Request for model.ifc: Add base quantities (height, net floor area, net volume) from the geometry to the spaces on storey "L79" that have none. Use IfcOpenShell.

First a look at what the model holds.

```python
import ifcopenshell
import ifcopenshell.util.element
import ifcopenshell.util.unit

model = ifcopenshell.open("model.ifc")
print(model.schema)
for unit_type in ("LENGTHUNIT", "AREAUNIT", "VOLUMEUNIT"):
    print(unit_type, ifcopenshell.util.unit.calculate_unit_scale(model, unit_type))
storey = next(s for s in model.by_type("IfcBuildingStorey") if s.Name == "L79")
spaces = [e for e in ifcopenshell.util.element.get_decomposition(storey) if e.is_a("IfcSpace")]
for e in sorted(spaces, key=lambda e: e.id()):
    print(e.id(), e.is_a(), e.Name, list(ifcopenshell.util.element.get_psets(e, qtos_only=True)), sep=" | ")
```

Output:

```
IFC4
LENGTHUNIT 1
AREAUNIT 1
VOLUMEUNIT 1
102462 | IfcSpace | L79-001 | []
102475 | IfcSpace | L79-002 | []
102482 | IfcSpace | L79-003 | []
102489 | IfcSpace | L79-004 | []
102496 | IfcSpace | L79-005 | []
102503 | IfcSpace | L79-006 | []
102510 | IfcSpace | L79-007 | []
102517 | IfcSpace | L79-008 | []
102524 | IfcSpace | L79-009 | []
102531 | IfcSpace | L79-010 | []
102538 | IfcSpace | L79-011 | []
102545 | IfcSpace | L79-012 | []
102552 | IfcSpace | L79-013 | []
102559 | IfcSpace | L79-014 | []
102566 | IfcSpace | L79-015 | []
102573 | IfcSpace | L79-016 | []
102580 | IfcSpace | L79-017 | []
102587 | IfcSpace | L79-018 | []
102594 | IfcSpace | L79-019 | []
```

```python
import ifcopenshell
import ifcopenshell.api.pset
import ifcopenshell.geom
import ifcopenshell.util.element
import ifcopenshell.util.shape
import ifcopenshell.util.unit

model = ifcopenshell.open("model.ifc")
unit_scale = ifcopenshell.util.unit.calculate_unit_scale(model)
area_scale = ifcopenshell.util.unit.calculate_unit_scale(model, "AREAUNIT")
volume_scale = ifcopenshell.util.unit.calculate_unit_scale(model, "VOLUMEUNIT")
settings = ifcopenshell.geom.settings()

storey = next(s for s in model.by_type("IfcBuildingStorey") if s.Name == "L79")
spaces = [e for e in ifcopenshell.util.element.get_decomposition(storey) if e.is_a("IfcSpace")]

for e in sorted(spaces, key=lambda e: e.id()):
    if ifcopenshell.util.element.get_psets(e, qtos_only=True, should_inherit=False):
        continue
    # Geometry comes back in metres, in the element's own axes.
    shape = ifcopenshell.geom.create_shape(settings, e)
    values = {
        "Height": ifcopenshell.util.shape.get_z(shape.geometry) / unit_scale,
        "NetFloorArea": ifcopenshell.util.shape.get_footprint_area(shape.geometry) / area_scale,
        "NetVolume": ifcopenshell.util.shape.get_volume(shape.geometry) / volume_scale,
    }
    qto = ifcopenshell.api.pset.add_qto(model, product=e, name="Qto_SpaceBaseQuantities")
    ifcopenshell.api.pset.edit_qto(model, qto=qto, properties=values)
    print(e.id(), {k: round(v, 3) for k, v in values.items()})

model.write("model_edited.ifc")
```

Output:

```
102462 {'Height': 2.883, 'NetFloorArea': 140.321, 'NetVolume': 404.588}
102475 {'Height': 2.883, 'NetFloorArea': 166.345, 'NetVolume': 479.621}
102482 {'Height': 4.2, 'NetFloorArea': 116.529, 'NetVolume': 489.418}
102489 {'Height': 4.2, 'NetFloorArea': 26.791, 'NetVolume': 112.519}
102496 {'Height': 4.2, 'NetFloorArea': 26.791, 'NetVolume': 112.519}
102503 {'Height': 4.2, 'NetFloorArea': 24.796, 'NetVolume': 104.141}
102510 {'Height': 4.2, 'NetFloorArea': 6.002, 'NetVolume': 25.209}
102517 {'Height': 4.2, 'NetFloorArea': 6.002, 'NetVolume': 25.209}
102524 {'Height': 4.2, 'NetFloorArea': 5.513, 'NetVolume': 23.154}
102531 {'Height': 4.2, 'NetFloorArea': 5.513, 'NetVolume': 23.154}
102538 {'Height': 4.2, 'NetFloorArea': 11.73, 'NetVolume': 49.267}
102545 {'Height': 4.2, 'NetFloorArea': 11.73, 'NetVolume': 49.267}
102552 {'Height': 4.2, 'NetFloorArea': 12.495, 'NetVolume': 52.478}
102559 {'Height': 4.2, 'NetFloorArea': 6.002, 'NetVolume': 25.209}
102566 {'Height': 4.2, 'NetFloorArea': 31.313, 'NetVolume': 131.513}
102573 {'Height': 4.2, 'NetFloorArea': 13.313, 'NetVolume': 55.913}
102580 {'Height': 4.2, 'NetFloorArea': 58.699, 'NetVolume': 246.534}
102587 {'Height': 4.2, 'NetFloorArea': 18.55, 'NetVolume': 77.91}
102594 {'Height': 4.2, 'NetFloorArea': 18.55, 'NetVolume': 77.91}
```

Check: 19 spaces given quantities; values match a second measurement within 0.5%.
